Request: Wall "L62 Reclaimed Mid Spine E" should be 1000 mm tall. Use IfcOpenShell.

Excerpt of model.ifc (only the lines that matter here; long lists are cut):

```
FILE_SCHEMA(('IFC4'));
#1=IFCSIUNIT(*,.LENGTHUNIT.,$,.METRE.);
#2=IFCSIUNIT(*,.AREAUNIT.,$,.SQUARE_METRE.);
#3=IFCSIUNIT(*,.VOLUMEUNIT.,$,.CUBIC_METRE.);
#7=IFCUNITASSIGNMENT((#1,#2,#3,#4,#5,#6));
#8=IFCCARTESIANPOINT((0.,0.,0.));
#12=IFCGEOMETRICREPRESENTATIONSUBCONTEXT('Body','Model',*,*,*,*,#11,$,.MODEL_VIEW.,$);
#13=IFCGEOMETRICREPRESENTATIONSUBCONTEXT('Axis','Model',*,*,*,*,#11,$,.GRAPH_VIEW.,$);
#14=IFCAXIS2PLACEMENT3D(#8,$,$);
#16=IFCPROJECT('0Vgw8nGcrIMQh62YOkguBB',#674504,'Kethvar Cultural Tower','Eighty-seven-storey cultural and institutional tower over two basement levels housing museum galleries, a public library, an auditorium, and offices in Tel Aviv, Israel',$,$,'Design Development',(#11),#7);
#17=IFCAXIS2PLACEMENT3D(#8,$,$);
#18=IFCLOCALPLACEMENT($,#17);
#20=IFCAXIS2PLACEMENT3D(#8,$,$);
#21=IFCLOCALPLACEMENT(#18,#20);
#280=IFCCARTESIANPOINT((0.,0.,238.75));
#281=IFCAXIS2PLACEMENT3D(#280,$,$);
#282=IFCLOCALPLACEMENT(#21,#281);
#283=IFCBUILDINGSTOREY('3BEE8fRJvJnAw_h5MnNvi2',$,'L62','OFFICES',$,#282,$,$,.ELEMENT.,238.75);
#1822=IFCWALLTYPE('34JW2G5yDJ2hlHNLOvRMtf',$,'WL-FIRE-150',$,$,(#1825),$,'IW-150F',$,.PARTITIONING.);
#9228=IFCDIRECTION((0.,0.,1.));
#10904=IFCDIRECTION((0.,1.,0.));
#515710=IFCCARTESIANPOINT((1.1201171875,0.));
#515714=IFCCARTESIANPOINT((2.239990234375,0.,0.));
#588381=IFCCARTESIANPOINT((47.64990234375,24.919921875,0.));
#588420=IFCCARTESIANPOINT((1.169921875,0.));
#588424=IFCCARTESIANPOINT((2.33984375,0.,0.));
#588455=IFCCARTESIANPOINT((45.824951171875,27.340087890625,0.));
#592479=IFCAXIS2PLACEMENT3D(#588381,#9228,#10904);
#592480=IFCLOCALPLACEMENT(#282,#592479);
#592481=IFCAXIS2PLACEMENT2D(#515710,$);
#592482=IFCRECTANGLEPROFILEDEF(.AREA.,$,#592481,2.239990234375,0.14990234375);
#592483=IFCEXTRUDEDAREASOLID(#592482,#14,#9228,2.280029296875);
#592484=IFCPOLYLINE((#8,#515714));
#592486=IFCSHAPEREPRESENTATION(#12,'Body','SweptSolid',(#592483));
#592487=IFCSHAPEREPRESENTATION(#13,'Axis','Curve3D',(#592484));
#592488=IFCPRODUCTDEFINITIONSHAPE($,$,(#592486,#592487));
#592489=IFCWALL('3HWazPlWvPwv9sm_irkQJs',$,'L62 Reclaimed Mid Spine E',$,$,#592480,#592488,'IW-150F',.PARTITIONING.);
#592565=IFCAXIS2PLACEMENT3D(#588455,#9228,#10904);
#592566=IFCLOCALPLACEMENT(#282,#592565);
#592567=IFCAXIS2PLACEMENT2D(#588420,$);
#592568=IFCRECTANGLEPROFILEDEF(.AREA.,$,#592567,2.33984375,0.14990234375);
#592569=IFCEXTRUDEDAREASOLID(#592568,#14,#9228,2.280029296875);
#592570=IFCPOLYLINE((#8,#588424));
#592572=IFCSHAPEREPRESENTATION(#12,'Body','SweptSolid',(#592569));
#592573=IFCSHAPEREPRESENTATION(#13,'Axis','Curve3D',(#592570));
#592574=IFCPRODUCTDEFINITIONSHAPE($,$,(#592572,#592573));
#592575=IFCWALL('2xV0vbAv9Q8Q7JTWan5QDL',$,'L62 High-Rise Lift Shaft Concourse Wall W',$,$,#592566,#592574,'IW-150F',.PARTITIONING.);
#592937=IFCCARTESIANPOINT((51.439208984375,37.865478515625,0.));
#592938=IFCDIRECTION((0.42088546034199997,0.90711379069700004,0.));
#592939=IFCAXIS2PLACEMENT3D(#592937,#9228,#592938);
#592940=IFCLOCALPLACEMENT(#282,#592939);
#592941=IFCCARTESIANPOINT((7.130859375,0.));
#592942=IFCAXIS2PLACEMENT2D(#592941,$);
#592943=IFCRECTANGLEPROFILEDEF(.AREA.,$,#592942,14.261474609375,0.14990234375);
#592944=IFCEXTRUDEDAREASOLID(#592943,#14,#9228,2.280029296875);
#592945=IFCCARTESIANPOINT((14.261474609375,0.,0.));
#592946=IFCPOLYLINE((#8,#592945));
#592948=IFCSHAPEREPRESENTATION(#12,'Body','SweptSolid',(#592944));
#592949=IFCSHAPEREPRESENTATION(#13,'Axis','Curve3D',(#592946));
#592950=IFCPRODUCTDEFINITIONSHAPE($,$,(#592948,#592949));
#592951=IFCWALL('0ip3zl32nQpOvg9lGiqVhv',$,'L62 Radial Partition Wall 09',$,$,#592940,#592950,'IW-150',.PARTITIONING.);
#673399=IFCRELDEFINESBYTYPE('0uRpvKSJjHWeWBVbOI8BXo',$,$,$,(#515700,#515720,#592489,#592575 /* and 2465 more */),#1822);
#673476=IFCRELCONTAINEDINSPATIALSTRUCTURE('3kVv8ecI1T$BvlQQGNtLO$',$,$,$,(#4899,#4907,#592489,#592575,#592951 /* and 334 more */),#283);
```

```python
import ifcopenshell
import ifcopenshell.geom
import ifcopenshell.util.representation
import ifcopenshell.util.shape

model = ifcopenshell.open("model.ifc")
settings = ifcopenshell.geom.settings()


def volume(element):
    """Net volume in cubic metres, openings subtracted."""
    shape = ifcopenshell.geom.create_shape(settings, element)
    return ifcopenshell.util.shape.get_volume(shape.geometry)


wall = model.by_guid("3HWazPlWvPwv9sm_irkQJs")
before = volume(wall)

body = ifcopenshell.util.representation.get_representation(wall, "Model", "Body")
solid = body.Items[0]
old_height = solid.Depth
solid.Depth = 1.0
after = volume(wall)

print(f"height {old_height:g} -> {solid.Depth:g}, volume {before:.3f} -> {after:.3f} m3")

model.write("model_v2.ifc")
```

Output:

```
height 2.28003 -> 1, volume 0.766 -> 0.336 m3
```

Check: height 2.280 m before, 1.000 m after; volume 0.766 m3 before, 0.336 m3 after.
